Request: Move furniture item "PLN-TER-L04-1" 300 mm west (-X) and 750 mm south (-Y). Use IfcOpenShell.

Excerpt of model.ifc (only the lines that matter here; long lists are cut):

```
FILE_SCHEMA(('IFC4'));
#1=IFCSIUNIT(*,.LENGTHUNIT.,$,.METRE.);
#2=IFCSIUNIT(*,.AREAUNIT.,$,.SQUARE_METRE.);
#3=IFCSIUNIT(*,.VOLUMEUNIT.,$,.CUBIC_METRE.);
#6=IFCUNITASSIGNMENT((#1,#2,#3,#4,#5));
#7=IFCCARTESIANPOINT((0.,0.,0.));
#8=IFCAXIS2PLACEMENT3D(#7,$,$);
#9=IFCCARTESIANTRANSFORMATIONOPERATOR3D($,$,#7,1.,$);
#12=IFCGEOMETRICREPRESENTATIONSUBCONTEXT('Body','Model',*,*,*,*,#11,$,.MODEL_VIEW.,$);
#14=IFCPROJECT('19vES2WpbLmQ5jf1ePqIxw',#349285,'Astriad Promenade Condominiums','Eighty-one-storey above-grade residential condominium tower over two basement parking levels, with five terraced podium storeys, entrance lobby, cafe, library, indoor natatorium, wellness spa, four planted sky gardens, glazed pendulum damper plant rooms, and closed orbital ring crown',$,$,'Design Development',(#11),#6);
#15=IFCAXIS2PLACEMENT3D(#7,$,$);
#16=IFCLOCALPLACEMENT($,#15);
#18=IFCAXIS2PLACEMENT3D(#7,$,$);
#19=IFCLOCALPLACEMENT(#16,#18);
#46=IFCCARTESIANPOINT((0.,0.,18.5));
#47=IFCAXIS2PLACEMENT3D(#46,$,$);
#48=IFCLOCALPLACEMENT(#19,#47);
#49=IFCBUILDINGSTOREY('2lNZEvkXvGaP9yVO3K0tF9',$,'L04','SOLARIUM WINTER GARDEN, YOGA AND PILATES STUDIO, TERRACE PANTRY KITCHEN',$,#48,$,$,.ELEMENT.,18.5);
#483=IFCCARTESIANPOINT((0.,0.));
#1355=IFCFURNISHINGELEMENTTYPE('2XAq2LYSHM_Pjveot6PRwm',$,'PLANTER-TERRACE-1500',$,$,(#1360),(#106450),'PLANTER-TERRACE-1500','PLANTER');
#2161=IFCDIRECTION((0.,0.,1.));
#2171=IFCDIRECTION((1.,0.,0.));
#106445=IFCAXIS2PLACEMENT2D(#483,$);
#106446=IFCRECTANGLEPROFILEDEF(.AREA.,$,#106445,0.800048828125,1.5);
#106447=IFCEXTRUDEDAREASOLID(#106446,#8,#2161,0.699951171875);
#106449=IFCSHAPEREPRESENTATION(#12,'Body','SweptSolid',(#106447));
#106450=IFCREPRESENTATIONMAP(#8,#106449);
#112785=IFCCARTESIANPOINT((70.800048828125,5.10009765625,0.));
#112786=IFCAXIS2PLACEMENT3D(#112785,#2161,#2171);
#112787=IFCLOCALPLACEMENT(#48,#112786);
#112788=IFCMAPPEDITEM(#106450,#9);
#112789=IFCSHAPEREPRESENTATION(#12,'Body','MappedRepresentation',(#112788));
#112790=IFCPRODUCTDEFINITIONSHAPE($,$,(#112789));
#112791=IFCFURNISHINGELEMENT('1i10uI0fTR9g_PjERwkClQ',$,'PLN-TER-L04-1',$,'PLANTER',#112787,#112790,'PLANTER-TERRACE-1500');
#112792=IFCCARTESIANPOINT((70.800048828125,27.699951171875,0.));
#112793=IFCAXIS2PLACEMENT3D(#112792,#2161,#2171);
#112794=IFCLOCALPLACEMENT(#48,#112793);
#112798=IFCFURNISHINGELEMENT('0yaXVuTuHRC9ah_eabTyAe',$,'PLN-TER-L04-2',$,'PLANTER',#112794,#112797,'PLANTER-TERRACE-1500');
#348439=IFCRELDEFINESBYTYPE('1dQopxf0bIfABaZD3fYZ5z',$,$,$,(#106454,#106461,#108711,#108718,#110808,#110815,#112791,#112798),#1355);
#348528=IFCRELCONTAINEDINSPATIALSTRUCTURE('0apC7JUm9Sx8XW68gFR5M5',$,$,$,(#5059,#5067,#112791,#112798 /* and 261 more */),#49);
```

```python
import ifcopenshell
import ifcopenshell.api.geometry
import ifcopenshell.util.placement
import ifcopenshell.util.unit

model = ifcopenshell.open("model.ifc")
unit_scale = ifcopenshell.util.unit.calculate_unit_scale(model)

item = model.by_guid("1i10uI0fTR9g_PjERwkClQ")
matrix = ifcopenshell.util.placement.get_local_placement(item.ObjectPlacement)
matrix[0, 3] -= 0.3 / unit_scale
matrix[1, 3] -= 0.75 / unit_scale
ifcopenshell.api.geometry.edit_object_placement(model, product=item, matrix=matrix, is_si=False)

print(ifcopenshell.util.placement.get_local_placement(item.ObjectPlacement).round(3) + 0.0)

model.write("model_updated.ifc")
```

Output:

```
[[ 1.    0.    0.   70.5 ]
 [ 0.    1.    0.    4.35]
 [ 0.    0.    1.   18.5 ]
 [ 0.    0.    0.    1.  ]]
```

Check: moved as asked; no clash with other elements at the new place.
